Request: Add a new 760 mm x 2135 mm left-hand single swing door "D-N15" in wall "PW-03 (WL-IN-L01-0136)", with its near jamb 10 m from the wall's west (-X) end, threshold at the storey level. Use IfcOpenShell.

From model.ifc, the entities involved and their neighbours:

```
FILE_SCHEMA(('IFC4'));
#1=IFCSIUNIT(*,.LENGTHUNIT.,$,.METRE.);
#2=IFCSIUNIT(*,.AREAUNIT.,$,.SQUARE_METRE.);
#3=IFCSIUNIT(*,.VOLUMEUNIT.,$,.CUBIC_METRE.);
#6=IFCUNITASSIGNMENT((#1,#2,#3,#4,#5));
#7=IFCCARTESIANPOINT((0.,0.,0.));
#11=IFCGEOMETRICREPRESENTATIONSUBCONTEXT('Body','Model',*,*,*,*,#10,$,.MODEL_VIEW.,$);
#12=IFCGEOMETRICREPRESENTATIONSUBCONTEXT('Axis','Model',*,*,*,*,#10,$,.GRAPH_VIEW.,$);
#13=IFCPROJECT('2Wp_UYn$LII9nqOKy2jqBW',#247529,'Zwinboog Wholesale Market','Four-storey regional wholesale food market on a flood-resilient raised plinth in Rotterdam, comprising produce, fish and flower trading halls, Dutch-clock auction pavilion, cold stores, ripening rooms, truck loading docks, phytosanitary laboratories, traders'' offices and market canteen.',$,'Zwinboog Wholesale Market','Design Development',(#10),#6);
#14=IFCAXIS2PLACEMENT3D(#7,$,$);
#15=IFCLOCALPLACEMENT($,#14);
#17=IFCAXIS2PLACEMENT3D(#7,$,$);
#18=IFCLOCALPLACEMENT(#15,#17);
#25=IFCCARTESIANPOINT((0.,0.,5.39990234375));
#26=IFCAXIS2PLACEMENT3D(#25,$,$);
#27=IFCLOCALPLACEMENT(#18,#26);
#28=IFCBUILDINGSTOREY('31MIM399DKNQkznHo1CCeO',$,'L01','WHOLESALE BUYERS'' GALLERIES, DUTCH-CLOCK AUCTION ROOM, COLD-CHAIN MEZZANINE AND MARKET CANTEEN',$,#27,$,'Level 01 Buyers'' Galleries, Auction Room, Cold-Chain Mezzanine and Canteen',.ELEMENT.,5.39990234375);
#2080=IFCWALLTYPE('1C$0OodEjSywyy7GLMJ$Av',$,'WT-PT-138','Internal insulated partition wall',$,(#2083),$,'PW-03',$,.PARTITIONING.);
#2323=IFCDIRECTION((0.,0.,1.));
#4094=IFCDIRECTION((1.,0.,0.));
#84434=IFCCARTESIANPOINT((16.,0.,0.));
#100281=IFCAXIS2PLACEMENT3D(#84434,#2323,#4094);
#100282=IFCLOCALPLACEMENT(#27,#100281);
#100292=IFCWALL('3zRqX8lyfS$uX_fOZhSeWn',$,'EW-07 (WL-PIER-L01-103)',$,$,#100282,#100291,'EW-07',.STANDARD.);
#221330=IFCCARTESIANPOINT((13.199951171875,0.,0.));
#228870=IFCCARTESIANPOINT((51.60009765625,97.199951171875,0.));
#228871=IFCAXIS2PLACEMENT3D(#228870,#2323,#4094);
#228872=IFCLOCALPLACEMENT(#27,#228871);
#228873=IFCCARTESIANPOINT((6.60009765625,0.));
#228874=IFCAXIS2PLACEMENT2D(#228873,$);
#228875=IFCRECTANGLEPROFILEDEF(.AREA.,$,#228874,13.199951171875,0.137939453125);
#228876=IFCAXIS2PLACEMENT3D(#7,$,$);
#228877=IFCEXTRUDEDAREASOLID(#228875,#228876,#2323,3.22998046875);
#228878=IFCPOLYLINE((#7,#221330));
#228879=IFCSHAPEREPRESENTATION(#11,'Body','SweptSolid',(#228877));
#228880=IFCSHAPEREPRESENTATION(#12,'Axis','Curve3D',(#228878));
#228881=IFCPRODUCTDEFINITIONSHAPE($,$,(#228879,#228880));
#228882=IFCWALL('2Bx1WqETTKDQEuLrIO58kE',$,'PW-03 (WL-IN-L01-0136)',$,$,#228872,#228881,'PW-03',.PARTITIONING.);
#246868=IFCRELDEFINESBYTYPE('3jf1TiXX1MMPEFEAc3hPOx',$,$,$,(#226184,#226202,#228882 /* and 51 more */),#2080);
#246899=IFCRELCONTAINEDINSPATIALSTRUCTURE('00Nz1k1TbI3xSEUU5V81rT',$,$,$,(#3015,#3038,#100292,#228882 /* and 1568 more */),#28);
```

```python
import numpy as np
import ifcopenshell
import ifcopenshell.api.feature
import ifcopenshell.api.geometry
import ifcopenshell.api.root
import ifcopenshell.api.spatial
import ifcopenshell.geom
import ifcopenshell.util.element
import ifcopenshell.util.placement
import ifcopenshell.util.representation
import ifcopenshell.util.shape
import ifcopenshell.util.unit

model = ifcopenshell.open("model.ifc")
unit_scale = ifcopenshell.util.unit.calculate_unit_scale(model)
settings = ifcopenshell.geom.settings()


def volume(element):
    """Net volume in cubic metres, openings subtracted."""
    shape = ifcopenshell.geom.create_shape(settings, element)
    return ifcopenshell.util.shape.get_volume(shape.geometry)


wall = model.by_guid("2Bx1WqETTKDQEuLrIO58kE")
storey = ifcopenshell.util.element.get_container(wall, ifc_class="IfcBuildingStorey")
context = ifcopenshell.util.representation.get_context(model, "Model", "Body", "MODEL_VIEW")
before = volume(wall)

width, height, from_end, sill = 0.76, 2.135, 10, 0.0  # metres

# The wall runs along its own X axis, and the end named is its -X end.
wall_shape = ifcopenshell.geom.create_shape(settings, wall)
x, y, z = ifcopenshell.util.shape.get_vertices(wall_shape.geometry).T
start = x.min() + from_end
face, thickness = float(y.min()), float(y.max() - y.min())
wall_matrix = ifcopenshell.util.placement.get_local_placement(wall.ObjectPlacement)
level = ifcopenshell.util.placement.get_local_placement(storey.ObjectPlacement)[2, 3]


def in_wall(x, y):
    """Placement at x, y metres in the wall's axes, at sill height."""
    matrix = wall_matrix.copy()
    matrix[:, 3] = wall_matrix @ np.array([x / unit_scale, y / unit_scale, 0.0, 1.0])
    matrix[2, 3] = level + sill / unit_scale
    return matrix


# Opening: a box that overshoots both wall faces by 50 mm.
opening = ifcopenshell.api.root.create_entity(model, ifc_class="IfcOpeningElement", predefined_type="OPENING")
box = ifcopenshell.api.geometry.add_wall_representation(
    model, context=context, length=width, height=height, thickness=thickness + 0.1
)
ifcopenshell.api.geometry.assign_representation(model, product=opening, representation=box)
ifcopenshell.api.geometry.edit_object_placement(model, product=opening, matrix=in_wall(start, face - 0.05), is_si=False)
ifcopenshell.api.feature.add_feature(model, feature=opening, element=wall)

door = ifcopenshell.api.root.create_entity(model, ifc_class="IfcDoor", name="D-N15", predefined_type="DOOR")
door.OverallWidth, door.OverallHeight = width / unit_scale, height / unit_scale
door.OperationType = "SINGLE_SWING_LEFT"
body = ifcopenshell.api.geometry.add_door_representation(
    model,
    context=context,
    overall_width=door.OverallWidth,
    overall_height=door.OverallHeight,
    operation_type="SINGLE_SWING_LEFT",
    lining_properties={"LiningDepth": thickness / unit_scale, "ThresholdDepth": thickness / unit_scale},
)
ifcopenshell.api.geometry.assign_representation(model, product=door, representation=body)
ifcopenshell.api.spatial.assign_container(model, products=[door], relating_structure=storey)
ifcopenshell.api.feature.add_filling(model, opening=opening, element=door)

# The lining spans the wall, so the door starts at the wall face.
ifcopenshell.api.geometry.edit_object_placement(model, product=door, matrix=in_wall(start, face), is_si=False)

after = volume(wall)

print(f"wall volume {before:.3f} -> {after:.3f} m3")

model.write("model_updated.ifc")
```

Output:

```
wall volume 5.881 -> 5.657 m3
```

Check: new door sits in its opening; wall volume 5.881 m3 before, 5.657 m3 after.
